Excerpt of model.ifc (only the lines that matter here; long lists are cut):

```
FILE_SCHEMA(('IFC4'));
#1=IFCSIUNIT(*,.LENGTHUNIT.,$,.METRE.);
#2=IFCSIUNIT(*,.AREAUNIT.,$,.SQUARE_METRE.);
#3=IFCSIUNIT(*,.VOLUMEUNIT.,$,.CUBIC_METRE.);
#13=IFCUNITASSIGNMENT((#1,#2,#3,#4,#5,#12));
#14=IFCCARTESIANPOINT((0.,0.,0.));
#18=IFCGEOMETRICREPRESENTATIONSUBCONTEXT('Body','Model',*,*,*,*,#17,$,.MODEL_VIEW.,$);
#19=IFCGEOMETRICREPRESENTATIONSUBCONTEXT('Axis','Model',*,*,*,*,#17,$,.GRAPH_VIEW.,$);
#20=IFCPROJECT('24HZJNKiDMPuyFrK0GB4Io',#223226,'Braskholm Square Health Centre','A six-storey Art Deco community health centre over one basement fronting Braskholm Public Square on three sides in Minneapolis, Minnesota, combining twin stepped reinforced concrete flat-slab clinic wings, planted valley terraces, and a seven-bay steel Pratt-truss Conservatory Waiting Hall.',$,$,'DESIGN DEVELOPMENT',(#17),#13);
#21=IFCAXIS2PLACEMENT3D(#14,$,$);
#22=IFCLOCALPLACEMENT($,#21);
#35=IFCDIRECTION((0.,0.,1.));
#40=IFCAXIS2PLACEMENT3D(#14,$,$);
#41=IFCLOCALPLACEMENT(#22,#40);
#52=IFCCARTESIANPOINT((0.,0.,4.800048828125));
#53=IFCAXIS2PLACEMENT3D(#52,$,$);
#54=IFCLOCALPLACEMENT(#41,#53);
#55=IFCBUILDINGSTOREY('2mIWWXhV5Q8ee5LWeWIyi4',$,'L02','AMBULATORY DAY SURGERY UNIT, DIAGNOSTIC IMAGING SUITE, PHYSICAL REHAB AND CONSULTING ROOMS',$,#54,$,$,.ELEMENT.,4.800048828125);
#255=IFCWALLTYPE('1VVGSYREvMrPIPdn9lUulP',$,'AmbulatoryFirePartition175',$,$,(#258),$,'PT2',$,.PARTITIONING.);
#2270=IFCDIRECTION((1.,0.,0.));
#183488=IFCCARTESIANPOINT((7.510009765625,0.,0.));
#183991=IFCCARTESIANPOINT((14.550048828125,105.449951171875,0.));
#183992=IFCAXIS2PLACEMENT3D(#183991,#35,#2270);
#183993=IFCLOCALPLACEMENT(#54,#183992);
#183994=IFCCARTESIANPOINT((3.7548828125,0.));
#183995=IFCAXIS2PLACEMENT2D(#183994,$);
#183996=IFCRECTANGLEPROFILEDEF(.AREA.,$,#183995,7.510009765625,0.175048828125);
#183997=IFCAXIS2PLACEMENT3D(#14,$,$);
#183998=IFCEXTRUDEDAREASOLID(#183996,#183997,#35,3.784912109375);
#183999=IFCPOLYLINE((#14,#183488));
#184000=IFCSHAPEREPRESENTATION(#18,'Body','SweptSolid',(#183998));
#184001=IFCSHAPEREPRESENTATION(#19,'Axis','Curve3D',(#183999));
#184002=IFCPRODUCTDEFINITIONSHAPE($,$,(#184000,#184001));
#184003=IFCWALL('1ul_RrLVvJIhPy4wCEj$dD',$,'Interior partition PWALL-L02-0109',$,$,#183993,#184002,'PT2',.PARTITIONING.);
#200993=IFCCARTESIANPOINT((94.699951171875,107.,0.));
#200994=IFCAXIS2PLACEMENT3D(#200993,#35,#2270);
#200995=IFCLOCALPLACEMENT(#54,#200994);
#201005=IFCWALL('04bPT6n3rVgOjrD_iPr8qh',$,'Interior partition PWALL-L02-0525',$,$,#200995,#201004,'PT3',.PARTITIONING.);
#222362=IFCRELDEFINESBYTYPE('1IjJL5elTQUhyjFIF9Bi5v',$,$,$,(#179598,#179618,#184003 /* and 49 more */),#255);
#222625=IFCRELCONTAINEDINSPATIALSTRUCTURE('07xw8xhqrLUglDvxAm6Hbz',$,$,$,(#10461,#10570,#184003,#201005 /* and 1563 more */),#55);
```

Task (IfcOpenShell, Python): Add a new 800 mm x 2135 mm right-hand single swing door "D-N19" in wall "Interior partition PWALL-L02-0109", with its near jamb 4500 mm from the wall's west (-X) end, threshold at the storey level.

```python
import numpy as np
import ifcopenshell
import ifcopenshell.api.feature
import ifcopenshell.api.geometry
import ifcopenshell.api.root
import ifcopenshell.api.spatial
import ifcopenshell.geom
import ifcopenshell.util.element
import ifcopenshell.util.placement
import ifcopenshell.util.representation
import ifcopenshell.util.shape
import ifcopenshell.util.unit

model = ifcopenshell.open("model.ifc")
unit_scale = ifcopenshell.util.unit.calculate_unit_scale(model)
settings = ifcopenshell.geom.settings()


def volume(element):
    """Net volume in cubic metres, openings subtracted."""
    shape = ifcopenshell.geom.create_shape(settings, element)
    return ifcopenshell.util.shape.get_volume(shape.geometry)


wall = model.by_guid("1ul_RrLVvJIhPy4wCEj$dD")
storey = ifcopenshell.util.element.get_container(wall, ifc_class="IfcBuildingStorey")
context = ifcopenshell.util.representation.get_context(model, "Model", "Body", "MODEL_VIEW")
before = volume(wall)

width, height, from_end, sill = 0.8, 2.135, 4.5, 0.0  # metres

# The wall runs along its own X axis, and the end named is its -X end.
wall_shape = ifcopenshell.geom.create_shape(settings, wall)
x, y, z = ifcopenshell.util.shape.get_vertices(wall_shape.geometry).T
start = x.min() + from_end
face, thickness = float(y.min()), float(y.max() - y.min())
wall_matrix = ifcopenshell.util.placement.get_local_placement(wall.ObjectPlacement)
level = ifcopenshell.util.placement.get_local_placement(storey.ObjectPlacement)[2, 3]


def in_wall(x, y):
    """Placement at x, y metres in the wall's axes, at sill height."""
    matrix = wall_matrix.copy()
    matrix[:, 3] = wall_matrix @ np.array([x / unit_scale, y / unit_scale, 0.0, 1.0])
    matrix[2, 3] = level + sill / unit_scale
    return matrix


# Opening: a box that overshoots both wall faces by 50 mm.
opening = ifcopenshell.api.root.create_entity(model, ifc_class="IfcOpeningElement", predefined_type="OPENING")
box = ifcopenshell.api.geometry.add_wall_representation(
    model, context=context, length=width, height=height, thickness=thickness + 0.1
)
ifcopenshell.api.geometry.assign_representation(model, product=opening, representation=box)
ifcopenshell.api.geometry.edit_object_placement(model, product=opening, matrix=in_wall(start, face - 0.05), is_si=False)
ifcopenshell.api.feature.add_feature(model, feature=opening, element=wall)

door = ifcopenshell.api.root.create_entity(model, ifc_class="IfcDoor", name="D-N19", predefined_type="DOOR")
door.OverallWidth, door.OverallHeight = width / unit_scale, height / unit_scale
door.OperationType = "SINGLE_SWING_RIGHT"
body = ifcopenshell.api.geometry.add_door_representation(
    model,
    context=context,
    overall_width=door.OverallWidth,
    overall_height=door.OverallHeight,
    operation_type="SINGLE_SWING_RIGHT",
    lining_properties={"LiningDepth": thickness / unit_scale, "ThresholdDepth": thickness / unit_scale},
)
ifcopenshell.api.geometry.assign_representation(model, product=door, representation=body)
ifcopenshell.api.spatial.assign_container(model, products=[door], relating_structure=storey)
ifcopenshell.api.feature.add_filling(model, opening=opening, element=door)

# The lining spans the wall, so the door starts at the wall face.
ifcopenshell.api.geometry.edit_object_placement(model, product=door, matrix=in_wall(start, face), is_si=False)

after = volume(wall)

print(f"wall volume {before:.3f} -> {after:.3f} m3")

model.write("model_updated.ifc")
```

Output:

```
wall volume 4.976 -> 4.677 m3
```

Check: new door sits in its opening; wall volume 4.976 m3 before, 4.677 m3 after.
